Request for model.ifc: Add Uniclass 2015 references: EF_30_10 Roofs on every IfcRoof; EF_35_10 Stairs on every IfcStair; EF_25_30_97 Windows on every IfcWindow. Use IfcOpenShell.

First a look at what the model holds.

```python
import ifcopenshell

model = ifcopenshell.open("model.ifc")
print(model.schema)
print("classifications:", [c.Name for c in model.by_type("IfcClassification")])
for ifc_class in ("IfcDoor", "IfcRoof", "IfcStair", "IfcWall", "IfcWindow"):
    print(ifc_class, len(model.by_type(ifc_class)))
```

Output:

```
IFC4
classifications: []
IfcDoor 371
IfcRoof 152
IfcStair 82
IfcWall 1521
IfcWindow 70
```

```python
import ifcopenshell
import ifcopenshell.api.classification

model = ifcopenshell.open("model.ifc")

system = ifcopenshell.api.classification.add_classification(model, classification="Uniclass 2015")

codes = {
    "IfcRoof": ("EF_30_10", "Roofs"),
    "IfcStair": ("EF_35_10", "Stairs"),
    "IfcWindow": ("EF_25_30_97", "Windows"),
}
for ifc_class, (code, name) in codes.items():
    products = model.by_type(ifc_class)
    ifcopenshell.api.classification.add_reference(
        model, products=products, classification=system, identification=code, name=name
    )
    print(code, len(products))

model.write("model_updated.ifc")
```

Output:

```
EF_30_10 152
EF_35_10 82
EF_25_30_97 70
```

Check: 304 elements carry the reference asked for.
